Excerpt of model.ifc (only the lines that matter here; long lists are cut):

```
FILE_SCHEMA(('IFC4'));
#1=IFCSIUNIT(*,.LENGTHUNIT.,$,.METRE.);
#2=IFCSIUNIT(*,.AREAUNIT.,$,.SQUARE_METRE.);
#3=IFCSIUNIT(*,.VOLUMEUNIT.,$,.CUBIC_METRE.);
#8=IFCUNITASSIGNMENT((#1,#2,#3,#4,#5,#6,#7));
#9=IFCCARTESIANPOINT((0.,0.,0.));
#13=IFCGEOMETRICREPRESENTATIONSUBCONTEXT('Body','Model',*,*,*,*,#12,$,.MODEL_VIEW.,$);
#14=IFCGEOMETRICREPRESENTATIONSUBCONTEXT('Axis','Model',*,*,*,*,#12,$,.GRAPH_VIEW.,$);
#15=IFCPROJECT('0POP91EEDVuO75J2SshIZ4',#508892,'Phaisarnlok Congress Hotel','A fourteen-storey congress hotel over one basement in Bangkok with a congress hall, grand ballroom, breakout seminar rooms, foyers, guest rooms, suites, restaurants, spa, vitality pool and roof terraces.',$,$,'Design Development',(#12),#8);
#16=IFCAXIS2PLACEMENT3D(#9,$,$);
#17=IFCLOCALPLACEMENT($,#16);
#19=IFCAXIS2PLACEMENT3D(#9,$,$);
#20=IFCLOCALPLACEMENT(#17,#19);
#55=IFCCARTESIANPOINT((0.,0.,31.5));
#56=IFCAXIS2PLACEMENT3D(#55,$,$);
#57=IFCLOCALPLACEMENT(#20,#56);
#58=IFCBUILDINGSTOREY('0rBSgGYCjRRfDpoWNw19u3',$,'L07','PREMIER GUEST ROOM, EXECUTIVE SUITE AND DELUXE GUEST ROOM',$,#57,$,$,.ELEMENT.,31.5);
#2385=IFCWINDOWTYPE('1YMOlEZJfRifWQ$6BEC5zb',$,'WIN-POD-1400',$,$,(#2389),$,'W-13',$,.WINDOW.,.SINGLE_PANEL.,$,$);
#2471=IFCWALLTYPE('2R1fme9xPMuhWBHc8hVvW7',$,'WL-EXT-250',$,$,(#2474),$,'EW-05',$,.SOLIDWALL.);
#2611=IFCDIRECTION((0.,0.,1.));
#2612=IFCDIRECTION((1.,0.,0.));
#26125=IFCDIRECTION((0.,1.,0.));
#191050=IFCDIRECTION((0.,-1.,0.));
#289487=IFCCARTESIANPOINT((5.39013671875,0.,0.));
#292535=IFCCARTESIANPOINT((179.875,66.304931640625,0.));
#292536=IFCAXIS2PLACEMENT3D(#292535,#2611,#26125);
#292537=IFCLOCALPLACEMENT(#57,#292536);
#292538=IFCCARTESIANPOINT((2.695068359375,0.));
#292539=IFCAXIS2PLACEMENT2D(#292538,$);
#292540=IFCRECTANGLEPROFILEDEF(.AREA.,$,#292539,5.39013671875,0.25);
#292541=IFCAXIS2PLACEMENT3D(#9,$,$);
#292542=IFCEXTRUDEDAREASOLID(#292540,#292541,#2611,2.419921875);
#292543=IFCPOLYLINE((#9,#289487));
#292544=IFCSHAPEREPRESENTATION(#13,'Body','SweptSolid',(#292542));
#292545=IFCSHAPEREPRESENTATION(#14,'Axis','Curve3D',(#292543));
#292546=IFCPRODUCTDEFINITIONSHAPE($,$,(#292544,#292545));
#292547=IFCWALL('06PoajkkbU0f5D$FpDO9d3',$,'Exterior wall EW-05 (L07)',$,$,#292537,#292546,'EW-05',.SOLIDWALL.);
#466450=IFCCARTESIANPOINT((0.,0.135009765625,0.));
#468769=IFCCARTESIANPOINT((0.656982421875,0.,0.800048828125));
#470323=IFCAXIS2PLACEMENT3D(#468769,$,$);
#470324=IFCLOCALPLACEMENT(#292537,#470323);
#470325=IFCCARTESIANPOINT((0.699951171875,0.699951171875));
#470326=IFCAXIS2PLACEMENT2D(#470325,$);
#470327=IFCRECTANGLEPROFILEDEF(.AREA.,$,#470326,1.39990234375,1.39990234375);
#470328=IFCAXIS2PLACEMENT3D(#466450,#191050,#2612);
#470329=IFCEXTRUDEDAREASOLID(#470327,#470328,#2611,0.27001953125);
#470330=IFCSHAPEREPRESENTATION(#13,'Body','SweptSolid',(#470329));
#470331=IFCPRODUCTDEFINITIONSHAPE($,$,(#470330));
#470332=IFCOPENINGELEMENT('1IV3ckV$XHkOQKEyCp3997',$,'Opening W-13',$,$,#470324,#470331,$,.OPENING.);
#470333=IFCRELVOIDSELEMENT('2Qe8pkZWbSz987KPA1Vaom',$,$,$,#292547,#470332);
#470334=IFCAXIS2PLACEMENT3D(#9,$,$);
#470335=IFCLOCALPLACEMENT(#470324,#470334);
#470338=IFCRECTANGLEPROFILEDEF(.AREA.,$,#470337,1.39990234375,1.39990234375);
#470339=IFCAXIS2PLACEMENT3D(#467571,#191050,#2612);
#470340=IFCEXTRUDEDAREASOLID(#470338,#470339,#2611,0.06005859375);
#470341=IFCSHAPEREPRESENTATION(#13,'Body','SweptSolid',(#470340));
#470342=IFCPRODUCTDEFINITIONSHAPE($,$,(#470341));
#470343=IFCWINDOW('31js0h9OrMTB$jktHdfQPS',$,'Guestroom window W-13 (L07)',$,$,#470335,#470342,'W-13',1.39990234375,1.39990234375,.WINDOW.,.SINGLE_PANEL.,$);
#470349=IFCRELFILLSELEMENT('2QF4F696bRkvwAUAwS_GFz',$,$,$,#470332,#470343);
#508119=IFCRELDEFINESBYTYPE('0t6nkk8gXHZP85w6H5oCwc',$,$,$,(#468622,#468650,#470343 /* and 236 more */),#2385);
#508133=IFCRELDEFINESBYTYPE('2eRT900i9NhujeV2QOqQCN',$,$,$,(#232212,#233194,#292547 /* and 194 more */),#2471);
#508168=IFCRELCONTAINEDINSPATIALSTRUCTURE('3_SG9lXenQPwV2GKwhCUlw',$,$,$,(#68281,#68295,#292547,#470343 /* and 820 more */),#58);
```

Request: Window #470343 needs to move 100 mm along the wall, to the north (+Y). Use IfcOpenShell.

```python
import ifcopenshell
import ifcopenshell.api.geometry
import ifcopenshell.util.placement
import ifcopenshell.util.unit

model = ifcopenshell.open("model.ifc")
unit_scale = ifcopenshell.util.unit.calculate_unit_scale(model)

window = model.by_guid("31js0h9OrMTB$jktHdfQPS")
opening = window.FillsVoids[0].RelatingOpeningElement
wall = opening.VoidsElements[0].RelatingBuildingElement

wall_matrix = ifcopenshell.util.placement.get_local_placement(wall.ObjectPlacement)
shift = wall_matrix[:3, 0] * 0.1 / unit_scale
before = ifcopenshell.util.placement.get_local_placement(window.ObjectPlacement)[:3, 3].copy()

# The window is placed relative to its opening, so it follows when the opening moves.
matrix = ifcopenshell.util.placement.get_local_placement(opening.ObjectPlacement)
matrix[:3, 3] += shift
ifcopenshell.api.geometry.edit_object_placement(
    model, product=opening, matrix=matrix, is_si=False, should_transform_children=True
)

after = ifcopenshell.util.placement.get_local_placement(window.ObjectPlacement)[:3, 3]
print("window moved by", (after - before).round(3) + 0.0)

model.write("model_v2.ifc")
```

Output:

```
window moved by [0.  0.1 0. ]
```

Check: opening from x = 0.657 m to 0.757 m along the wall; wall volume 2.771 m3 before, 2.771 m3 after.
